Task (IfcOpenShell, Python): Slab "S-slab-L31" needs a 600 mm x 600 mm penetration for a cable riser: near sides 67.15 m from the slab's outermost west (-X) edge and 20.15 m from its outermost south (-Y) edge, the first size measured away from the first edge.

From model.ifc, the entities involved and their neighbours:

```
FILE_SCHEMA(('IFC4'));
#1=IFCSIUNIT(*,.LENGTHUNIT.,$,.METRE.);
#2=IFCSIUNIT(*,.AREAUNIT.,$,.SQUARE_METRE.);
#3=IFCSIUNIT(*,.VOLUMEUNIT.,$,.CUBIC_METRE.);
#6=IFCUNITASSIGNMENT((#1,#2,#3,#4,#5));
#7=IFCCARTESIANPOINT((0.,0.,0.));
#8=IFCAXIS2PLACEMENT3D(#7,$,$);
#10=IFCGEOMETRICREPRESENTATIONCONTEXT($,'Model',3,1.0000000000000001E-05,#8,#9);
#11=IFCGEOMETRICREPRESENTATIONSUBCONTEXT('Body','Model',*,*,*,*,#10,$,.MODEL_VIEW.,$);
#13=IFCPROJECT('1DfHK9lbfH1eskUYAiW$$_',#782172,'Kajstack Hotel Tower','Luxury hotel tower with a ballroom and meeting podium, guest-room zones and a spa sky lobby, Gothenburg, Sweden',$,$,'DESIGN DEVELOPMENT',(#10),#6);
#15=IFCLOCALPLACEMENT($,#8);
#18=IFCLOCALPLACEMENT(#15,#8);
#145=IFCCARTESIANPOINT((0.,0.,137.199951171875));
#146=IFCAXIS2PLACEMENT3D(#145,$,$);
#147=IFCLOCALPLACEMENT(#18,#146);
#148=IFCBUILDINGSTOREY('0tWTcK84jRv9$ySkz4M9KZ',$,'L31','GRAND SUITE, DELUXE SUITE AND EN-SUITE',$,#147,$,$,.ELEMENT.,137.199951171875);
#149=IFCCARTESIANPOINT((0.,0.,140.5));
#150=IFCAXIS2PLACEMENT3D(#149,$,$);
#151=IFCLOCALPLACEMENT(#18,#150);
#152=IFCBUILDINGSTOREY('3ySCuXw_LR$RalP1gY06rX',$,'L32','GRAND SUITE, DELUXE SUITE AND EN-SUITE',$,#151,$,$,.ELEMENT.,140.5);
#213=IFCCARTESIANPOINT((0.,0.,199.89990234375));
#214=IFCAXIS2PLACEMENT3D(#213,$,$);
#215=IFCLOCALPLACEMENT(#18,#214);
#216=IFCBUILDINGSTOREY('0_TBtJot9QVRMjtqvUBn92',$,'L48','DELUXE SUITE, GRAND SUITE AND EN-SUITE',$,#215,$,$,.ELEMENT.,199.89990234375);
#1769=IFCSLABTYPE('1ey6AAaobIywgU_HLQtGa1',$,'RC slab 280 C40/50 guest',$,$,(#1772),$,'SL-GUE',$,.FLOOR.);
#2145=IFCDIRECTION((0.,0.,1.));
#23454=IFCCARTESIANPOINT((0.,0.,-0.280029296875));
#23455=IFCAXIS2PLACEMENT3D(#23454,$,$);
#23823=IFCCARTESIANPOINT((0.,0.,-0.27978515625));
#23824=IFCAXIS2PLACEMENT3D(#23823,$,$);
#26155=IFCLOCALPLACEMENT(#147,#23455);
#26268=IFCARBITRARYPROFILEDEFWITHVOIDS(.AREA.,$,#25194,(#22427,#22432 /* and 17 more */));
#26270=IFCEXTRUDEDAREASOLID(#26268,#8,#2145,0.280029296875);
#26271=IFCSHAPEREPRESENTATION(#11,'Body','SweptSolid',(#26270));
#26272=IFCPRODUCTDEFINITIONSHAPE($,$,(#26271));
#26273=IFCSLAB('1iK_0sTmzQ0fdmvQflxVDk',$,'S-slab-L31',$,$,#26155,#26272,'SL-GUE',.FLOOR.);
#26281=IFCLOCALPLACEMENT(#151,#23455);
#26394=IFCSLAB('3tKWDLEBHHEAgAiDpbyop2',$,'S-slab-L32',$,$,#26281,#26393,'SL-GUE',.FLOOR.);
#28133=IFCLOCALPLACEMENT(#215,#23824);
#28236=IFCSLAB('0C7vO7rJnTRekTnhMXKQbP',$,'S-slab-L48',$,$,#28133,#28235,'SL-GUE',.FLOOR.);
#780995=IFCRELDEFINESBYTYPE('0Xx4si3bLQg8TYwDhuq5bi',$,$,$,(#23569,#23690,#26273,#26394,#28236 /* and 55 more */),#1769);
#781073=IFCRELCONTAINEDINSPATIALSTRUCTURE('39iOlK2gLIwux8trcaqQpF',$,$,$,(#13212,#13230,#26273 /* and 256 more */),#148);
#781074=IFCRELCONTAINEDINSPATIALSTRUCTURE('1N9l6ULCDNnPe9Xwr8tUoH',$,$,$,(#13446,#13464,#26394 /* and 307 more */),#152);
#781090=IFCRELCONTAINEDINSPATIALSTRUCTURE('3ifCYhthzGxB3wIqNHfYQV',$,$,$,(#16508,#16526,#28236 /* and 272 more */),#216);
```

```python
import numpy as np
import ifcopenshell
import ifcopenshell.api.feature
import ifcopenshell.api.geometry
import ifcopenshell.api.root
import ifcopenshell.geom
import ifcopenshell.util.placement
import ifcopenshell.util.representation
import ifcopenshell.util.shape
import ifcopenshell.util.unit

model = ifcopenshell.open("model.ifc")
unit_scale = ifcopenshell.util.unit.calculate_unit_scale(model)
settings = ifcopenshell.geom.settings()


def volume(element):
    """Net volume in cubic metres, openings subtracted."""
    shape = ifcopenshell.geom.create_shape(settings, element)
    return ifcopenshell.util.shape.get_volume(shape.geometry)


slab = model.by_guid("1iK_0sTmzQ0fdmvQflxVDk")
before = volume(slab)

# Extent in the slab's own axes, in metres. The edges named are its -X and -Y sides.
slab_shape = ifcopenshell.geom.create_shape(settings, slab)
vertices = ifcopenshell.util.shape.get_vertices(slab_shape.geometry)
x_min, y_min, bottom = vertices.min(axis=0)
top = vertices[:, 2].max()

opening = ifcopenshell.api.root.create_entity(model, ifc_class="IfcOpeningElement", name="Cable riser opening", predefined_type="OPENING")
context = ifcopenshell.util.representation.get_context(model, "Model", "Body", "MODEL_VIEW")
width, depth = 0.6, 0.6
outline = [(0.0, 0.0), (width, 0.0), (width, depth), (0.0, depth), (0.0, 0.0)]
# Overshoot both faces by 50 mm so the cut is clean.
shape = ifcopenshell.api.geometry.add_slab_representation(
    model, context=context, depth=top - bottom + 0.1, polyline=outline
)
ifcopenshell.api.geometry.assign_representation(model, product=opening, representation=shape)

matrix = ifcopenshell.util.placement.get_local_placement(slab.ObjectPlacement)
matrix[:, 3] = matrix @ np.append(np.array([x_min + 67.15, y_min + 20.15, bottom - 0.05]) / unit_scale, 1.0)
ifcopenshell.api.geometry.edit_object_placement(model, product=opening, matrix=matrix, is_si=False)
ifcopenshell.api.feature.add_feature(model, feature=opening, element=slab)

after = volume(slab)

print(f"slab volume {before:.3f} -> {after:.3f} m3")

model.write("model_v2.ifc")
```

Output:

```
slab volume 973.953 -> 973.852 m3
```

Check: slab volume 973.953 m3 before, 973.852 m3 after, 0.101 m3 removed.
